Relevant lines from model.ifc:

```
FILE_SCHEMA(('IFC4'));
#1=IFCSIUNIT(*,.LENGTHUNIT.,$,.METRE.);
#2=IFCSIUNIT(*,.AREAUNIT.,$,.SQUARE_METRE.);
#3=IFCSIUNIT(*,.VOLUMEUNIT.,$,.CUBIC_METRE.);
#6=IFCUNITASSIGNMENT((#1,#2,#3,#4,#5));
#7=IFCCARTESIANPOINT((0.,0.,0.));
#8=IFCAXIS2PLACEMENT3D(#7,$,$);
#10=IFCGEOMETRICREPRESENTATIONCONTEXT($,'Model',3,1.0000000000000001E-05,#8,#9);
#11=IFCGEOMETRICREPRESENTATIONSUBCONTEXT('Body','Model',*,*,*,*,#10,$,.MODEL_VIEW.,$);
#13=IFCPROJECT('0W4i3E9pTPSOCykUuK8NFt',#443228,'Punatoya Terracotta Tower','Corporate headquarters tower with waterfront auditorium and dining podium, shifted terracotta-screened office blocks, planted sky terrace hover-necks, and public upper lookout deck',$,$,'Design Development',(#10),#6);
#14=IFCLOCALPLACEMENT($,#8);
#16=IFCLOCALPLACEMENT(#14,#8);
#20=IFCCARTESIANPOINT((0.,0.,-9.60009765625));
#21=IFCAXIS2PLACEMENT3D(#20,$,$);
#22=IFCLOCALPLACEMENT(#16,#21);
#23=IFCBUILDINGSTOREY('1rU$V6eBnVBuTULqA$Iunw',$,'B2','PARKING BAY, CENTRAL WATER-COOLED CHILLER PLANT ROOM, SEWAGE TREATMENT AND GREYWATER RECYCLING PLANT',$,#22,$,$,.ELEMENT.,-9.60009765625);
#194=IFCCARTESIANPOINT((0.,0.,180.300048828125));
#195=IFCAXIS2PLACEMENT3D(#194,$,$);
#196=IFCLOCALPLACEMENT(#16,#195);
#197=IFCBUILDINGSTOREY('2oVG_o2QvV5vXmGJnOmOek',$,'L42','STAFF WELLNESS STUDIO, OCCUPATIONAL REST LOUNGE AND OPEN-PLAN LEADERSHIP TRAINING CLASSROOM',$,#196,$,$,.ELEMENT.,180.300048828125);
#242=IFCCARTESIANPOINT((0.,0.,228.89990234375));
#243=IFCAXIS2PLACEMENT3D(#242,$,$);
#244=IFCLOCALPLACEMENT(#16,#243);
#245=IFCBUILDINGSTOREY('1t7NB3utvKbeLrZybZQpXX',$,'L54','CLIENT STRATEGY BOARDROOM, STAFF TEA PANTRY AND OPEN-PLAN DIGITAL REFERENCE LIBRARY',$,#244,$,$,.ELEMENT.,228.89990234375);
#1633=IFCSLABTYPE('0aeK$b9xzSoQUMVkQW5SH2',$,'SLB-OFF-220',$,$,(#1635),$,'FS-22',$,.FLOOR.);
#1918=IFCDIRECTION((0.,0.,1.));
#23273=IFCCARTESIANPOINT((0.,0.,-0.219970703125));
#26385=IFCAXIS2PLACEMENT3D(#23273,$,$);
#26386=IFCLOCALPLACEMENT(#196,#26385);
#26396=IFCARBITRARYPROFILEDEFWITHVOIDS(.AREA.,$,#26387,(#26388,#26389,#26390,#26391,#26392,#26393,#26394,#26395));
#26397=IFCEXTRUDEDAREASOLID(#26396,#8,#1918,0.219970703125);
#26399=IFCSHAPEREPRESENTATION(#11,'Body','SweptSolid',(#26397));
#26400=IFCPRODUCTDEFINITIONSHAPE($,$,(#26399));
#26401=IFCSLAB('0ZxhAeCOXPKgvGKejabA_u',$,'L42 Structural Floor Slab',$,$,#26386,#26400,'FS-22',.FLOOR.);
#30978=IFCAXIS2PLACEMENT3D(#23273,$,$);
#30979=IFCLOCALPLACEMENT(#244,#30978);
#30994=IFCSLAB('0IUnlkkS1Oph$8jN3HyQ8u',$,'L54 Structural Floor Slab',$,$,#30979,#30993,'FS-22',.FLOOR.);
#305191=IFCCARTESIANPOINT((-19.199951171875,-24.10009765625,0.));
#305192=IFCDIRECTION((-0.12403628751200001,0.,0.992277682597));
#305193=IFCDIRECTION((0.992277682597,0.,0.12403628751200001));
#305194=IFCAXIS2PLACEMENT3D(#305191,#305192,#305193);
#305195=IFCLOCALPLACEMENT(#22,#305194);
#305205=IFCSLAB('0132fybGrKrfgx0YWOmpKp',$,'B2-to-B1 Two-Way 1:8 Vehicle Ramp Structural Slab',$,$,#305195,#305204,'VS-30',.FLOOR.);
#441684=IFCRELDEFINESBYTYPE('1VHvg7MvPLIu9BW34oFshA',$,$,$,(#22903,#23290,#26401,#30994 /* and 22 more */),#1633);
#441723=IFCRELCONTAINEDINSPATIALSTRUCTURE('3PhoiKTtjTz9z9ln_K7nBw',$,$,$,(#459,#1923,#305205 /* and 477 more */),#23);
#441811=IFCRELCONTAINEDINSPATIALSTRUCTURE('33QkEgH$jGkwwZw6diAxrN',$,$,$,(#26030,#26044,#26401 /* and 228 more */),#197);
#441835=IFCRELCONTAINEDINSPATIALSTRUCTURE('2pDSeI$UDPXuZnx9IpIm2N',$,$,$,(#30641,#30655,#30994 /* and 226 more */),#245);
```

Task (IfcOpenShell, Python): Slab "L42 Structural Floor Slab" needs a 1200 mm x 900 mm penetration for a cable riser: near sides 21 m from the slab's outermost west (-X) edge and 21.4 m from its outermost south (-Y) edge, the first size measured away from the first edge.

```python
import numpy as np
import ifcopenshell
import ifcopenshell.api.feature
import ifcopenshell.api.geometry
import ifcopenshell.api.root
import ifcopenshell.geom
import ifcopenshell.util.placement
import ifcopenshell.util.representation
import ifcopenshell.util.shape
import ifcopenshell.util.unit

model = ifcopenshell.open("model.ifc")
unit_scale = ifcopenshell.util.unit.calculate_unit_scale(model)
settings = ifcopenshell.geom.settings()


def volume(element):
    """Net volume in cubic metres, openings subtracted."""
    shape = ifcopenshell.geom.create_shape(settings, element)
    return ifcopenshell.util.shape.get_volume(shape.geometry)


slab = model.by_guid("0ZxhAeCOXPKgvGKejabA_u")
before = volume(slab)

# Extent in the slab's own axes, in metres. The edges named are its -X and -Y sides.
slab_shape = ifcopenshell.geom.create_shape(settings, slab)
vertices = ifcopenshell.util.shape.get_vertices(slab_shape.geometry)
x_min, y_min, bottom = vertices.min(axis=0)
top = vertices[:, 2].max()

opening = ifcopenshell.api.root.create_entity(model, ifc_class="IfcOpeningElement", name="Cable riser opening", predefined_type="OPENING")
context = ifcopenshell.util.representation.get_context(model, "Model", "Body", "MODEL_VIEW")
width, depth = 1.2, 0.9
outline = [(0.0, 0.0), (width, 0.0), (width, depth), (0.0, depth), (0.0, 0.0)]
# Overshoot both faces by 50 mm so the cut is clean.
shape = ifcopenshell.api.geometry.add_slab_representation(
    model, context=context, depth=top - bottom + 0.1, polyline=outline
)
ifcopenshell.api.geometry.assign_representation(model, product=opening, representation=shape)

matrix = ifcopenshell.util.placement.get_local_placement(slab.ObjectPlacement)
matrix[:, 3] = matrix @ np.append(np.array([x_min + 21, y_min + 21.4, bottom - 0.05]) / unit_scale, 1.0)
ifcopenshell.api.geometry.edit_object_placement(model, product=opening, matrix=matrix, is_si=False)
ifcopenshell.api.feature.add_feature(model, feature=opening, element=slab)

after = volume(slab)

print(f"slab volume {before:.3f} -> {after:.3f} m3")

model.write("model_edited.ifc")
```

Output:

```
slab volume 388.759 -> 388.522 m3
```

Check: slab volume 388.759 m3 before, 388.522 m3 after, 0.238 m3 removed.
